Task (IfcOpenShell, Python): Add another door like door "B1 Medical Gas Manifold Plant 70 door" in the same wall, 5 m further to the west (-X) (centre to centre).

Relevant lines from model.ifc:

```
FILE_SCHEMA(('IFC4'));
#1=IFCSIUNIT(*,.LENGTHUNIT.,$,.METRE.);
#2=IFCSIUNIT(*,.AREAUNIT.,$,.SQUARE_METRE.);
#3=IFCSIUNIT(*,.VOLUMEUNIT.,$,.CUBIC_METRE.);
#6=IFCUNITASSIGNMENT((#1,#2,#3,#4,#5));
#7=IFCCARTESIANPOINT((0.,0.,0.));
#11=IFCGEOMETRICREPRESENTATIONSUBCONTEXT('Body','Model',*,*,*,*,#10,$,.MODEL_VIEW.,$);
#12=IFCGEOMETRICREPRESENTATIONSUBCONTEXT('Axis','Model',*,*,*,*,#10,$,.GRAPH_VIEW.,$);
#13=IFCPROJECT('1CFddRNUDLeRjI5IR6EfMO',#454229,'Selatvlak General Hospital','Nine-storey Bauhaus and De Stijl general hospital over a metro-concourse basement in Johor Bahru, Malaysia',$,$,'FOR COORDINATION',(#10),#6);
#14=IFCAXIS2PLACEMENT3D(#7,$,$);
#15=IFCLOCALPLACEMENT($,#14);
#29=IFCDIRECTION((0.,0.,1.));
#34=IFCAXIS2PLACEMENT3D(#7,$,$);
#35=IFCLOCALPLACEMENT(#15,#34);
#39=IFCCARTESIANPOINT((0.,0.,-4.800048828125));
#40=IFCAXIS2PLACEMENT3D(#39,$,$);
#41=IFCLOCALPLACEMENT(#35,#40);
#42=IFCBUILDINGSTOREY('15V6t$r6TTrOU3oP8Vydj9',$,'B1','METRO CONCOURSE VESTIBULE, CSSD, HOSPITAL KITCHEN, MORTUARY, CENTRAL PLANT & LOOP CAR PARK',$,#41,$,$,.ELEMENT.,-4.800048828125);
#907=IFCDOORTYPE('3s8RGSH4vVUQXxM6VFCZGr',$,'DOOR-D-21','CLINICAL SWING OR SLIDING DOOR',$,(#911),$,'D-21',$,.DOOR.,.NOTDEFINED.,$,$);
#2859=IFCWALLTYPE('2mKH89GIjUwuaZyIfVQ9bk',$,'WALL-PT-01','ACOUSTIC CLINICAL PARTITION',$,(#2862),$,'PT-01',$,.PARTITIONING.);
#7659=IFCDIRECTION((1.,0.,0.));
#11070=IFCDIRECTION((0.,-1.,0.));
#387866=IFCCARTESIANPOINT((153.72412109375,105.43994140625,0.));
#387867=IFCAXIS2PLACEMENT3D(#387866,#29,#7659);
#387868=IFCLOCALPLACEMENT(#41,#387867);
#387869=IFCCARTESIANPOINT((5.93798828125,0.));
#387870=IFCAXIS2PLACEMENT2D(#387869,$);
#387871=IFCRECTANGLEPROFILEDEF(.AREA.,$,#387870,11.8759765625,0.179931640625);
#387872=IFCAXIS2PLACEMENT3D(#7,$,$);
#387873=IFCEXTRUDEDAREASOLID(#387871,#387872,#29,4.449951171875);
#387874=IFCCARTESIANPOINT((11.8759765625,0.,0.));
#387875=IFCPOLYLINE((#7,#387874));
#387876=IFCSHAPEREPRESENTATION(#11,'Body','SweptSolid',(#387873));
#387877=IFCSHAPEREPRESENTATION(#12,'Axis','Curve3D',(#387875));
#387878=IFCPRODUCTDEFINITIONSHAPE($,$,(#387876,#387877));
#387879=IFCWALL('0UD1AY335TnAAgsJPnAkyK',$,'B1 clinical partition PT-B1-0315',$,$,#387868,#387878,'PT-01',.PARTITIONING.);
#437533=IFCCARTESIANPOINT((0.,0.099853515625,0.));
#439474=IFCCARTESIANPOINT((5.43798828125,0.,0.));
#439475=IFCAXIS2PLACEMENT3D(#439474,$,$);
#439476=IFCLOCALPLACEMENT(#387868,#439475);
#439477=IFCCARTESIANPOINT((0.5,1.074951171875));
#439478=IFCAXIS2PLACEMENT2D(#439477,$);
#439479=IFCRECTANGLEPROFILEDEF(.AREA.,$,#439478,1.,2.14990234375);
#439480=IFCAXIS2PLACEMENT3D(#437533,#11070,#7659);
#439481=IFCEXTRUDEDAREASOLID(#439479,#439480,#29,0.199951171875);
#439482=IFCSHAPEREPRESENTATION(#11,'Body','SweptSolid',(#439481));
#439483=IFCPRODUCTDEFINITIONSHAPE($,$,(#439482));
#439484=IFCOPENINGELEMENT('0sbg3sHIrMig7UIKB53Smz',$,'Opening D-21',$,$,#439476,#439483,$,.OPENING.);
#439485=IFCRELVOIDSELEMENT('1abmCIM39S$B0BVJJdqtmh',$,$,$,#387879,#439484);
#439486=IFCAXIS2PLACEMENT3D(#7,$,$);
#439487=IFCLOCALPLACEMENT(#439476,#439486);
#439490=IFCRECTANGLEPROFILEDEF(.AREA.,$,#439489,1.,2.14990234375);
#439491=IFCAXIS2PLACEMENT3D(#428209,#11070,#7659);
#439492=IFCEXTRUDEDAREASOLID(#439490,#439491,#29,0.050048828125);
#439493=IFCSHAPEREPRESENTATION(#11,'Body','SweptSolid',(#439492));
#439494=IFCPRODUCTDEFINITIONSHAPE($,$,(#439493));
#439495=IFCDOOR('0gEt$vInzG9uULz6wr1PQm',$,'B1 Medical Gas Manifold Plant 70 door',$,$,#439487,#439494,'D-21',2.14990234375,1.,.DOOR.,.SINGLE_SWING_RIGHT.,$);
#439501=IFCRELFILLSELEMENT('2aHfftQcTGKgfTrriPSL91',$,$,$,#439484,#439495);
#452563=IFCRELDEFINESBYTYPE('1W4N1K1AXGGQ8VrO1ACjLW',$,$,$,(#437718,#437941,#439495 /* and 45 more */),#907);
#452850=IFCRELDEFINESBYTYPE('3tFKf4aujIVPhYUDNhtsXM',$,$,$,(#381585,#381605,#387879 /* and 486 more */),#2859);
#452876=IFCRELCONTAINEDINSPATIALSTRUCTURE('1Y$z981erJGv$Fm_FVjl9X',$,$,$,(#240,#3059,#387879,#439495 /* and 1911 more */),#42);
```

```python
import ifcopenshell
import ifcopenshell.api.feature
import ifcopenshell.api.geometry
import ifcopenshell.api.root
import ifcopenshell.geom
import ifcopenshell.util.element
import ifcopenshell.util.placement
import ifcopenshell.util.shape
import ifcopenshell.util.unit

model = ifcopenshell.open("model.ifc")
unit_scale = ifcopenshell.util.unit.calculate_unit_scale(model)
settings = ifcopenshell.geom.settings()


def volume(element):
    """Net volume in cubic metres, openings subtracted."""
    shape = ifcopenshell.geom.create_shape(settings, element)
    return ifcopenshell.util.shape.get_volume(shape.geometry)


door = model.by_guid("0gEt$vInzG9uULz6wr1PQm")
opening = door.FillsVoids[0].RelatingOpeningElement
wall = opening.VoidsElements[0].RelatingBuildingElement
before = volume(wall)
shift = ifcopenshell.util.placement.get_local_placement(wall.ObjectPlacement)[:3, 0] * -5 / unit_scale

# copy_class copies the void relationship, type, container and properties, but no geometry.
new_opening = ifcopenshell.api.root.copy_class(model, product=opening)
new_opening.Representation = ifcopenshell.util.element.copy_deep(
    model, opening.Representation, exclude=["IfcGeometricRepresentationContext", "IfcRepresentationMap"]
)
new_door = ifcopenshell.api.root.copy_class(model, product=door)
new_door.Representation = ifcopenshell.util.element.copy_deep(
    model, door.Representation, exclude=["IfcGeometricRepresentationContext", "IfcRepresentationMap"]
)
new_door.Tag = None
ifcopenshell.api.feature.add_filling(model, opening=new_opening, element=new_door)

for old, new in ((opening, new_opening), (door, new_door)):
    matrix = ifcopenshell.util.placement.get_local_placement(old.ObjectPlacement)
    matrix[:3, 3] += shift
    ifcopenshell.api.geometry.edit_object_placement(model, product=new, matrix=matrix, is_si=False)

after = volume(wall)

print(f"wall volume {before:.3f} -> {after:.3f} m3")

model.write("model_updated.ifc")
```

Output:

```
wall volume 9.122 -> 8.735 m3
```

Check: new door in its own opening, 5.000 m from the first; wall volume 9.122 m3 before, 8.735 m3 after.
